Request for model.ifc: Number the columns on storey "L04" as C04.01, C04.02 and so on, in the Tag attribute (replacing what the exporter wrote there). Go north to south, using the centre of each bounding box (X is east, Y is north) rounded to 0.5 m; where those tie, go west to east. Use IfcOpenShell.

First a look at what the model holds.

```python
import ifcopenshell
import ifcopenshell.util.element
import ifcopenshell.util.placement

model = ifcopenshell.open("model.ifc")
print(model.schema)
storey = next(s for s in model.by_type("IfcBuildingStorey") if s.Name == "L04")
columns = [e for e in ifcopenshell.util.element.get_decomposition(storey) if e.is_a("IfcColumn")]
for e in sorted(columns, key=lambda e: e.id()):
    origin = ifcopenshell.util.placement.get_local_placement(e.ObjectPlacement)[:3, 3]
    print(e.id(), e.Tag, e.Name, origin.round(2) + 0.0, sep=" | ")
```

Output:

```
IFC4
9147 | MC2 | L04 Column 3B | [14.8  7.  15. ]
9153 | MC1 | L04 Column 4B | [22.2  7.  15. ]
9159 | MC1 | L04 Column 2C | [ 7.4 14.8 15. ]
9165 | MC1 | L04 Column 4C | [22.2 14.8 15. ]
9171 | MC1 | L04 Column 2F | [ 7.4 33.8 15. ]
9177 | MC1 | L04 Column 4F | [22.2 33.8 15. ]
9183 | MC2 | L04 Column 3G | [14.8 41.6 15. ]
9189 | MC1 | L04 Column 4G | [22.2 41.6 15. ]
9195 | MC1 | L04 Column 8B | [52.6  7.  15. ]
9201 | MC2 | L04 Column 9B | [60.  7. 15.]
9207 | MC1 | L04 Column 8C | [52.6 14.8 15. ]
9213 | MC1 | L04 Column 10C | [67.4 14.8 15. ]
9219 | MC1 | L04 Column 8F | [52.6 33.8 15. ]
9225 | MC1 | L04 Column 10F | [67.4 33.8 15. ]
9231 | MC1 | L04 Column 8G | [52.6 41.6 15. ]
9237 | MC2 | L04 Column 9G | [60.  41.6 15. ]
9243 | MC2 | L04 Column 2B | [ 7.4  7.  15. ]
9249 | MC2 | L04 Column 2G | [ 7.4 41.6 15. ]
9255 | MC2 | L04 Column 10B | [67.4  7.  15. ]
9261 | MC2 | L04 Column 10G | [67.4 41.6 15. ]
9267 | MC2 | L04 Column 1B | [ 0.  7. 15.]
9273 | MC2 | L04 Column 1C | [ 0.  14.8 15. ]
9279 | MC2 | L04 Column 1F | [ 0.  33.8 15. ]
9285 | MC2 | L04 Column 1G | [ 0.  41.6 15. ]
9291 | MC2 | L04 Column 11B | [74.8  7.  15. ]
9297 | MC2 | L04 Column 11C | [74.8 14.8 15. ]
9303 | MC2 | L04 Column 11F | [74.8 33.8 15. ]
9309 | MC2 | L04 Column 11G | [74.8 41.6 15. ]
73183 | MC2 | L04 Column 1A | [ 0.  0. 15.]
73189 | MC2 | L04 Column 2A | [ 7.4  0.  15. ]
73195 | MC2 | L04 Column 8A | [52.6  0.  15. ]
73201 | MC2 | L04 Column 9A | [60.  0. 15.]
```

```python
import ifcopenshell
import ifcopenshell.geom
import ifcopenshell.util.element
import ifcopenshell.util.shape

model = ifcopenshell.open("model.ifc")
settings = ifcopenshell.geom.settings()
settings.set("use-world-coords", True)


def centre(element):
    shape = ifcopenshell.geom.create_shape(settings, element)
    return ifcopenshell.util.shape.get_bbox_centroid(shape.geometry)


storey = next(s for s in model.by_type("IfcBuildingStorey") if s.Name == "L04")
columns = [e for e in ifcopenshell.util.element.get_decomposition(storey) if e.is_a("IfcColumn")]

# Insertion points can sit at a corner or the storey origin, so sort by the geometry (in metres).
centres = {e: centre(e) for e in columns}
columns.sort(key=lambda e: (-round(centres[e][1] / 0.5), centres[e][0]))

for i, e in enumerate(columns, start=1):
    number = f"C04.{i:02d}"
    e.Tag = number
    print(e.id(), number)

model.write("model_edited.ifc")
```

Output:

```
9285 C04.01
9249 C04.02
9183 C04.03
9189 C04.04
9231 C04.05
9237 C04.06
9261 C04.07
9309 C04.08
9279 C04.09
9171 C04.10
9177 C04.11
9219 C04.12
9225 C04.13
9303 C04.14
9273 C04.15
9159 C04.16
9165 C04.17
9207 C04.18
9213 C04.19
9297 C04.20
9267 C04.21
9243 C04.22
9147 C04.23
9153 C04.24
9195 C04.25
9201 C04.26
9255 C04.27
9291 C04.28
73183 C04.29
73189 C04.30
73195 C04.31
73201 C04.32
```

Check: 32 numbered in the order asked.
